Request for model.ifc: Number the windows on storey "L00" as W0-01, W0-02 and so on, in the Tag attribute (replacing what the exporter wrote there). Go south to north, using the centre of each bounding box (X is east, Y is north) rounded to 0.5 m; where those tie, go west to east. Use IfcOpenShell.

First a look at what the model holds.

```python
import ifcopenshell
import ifcopenshell.util.element
import ifcopenshell.util.placement

model = ifcopenshell.open("model.ifc")
print(model.schema)
storey = next(s for s in model.by_type("IfcBuildingStorey") if s.Name == "L00")
windows = [e for e in ifcopenshell.util.element.get_decomposition(storey) if e.is_a("IfcWindow")]
for e in sorted(windows, key=lambda e: e.id()):
    origin = ifcopenshell.util.placement.get_local_placement(e.ObjectPlacement)[:3, 3]
    print(e.id(), e.Tag, e.Name, origin.round(2) + 0.0, sep=" | ")
```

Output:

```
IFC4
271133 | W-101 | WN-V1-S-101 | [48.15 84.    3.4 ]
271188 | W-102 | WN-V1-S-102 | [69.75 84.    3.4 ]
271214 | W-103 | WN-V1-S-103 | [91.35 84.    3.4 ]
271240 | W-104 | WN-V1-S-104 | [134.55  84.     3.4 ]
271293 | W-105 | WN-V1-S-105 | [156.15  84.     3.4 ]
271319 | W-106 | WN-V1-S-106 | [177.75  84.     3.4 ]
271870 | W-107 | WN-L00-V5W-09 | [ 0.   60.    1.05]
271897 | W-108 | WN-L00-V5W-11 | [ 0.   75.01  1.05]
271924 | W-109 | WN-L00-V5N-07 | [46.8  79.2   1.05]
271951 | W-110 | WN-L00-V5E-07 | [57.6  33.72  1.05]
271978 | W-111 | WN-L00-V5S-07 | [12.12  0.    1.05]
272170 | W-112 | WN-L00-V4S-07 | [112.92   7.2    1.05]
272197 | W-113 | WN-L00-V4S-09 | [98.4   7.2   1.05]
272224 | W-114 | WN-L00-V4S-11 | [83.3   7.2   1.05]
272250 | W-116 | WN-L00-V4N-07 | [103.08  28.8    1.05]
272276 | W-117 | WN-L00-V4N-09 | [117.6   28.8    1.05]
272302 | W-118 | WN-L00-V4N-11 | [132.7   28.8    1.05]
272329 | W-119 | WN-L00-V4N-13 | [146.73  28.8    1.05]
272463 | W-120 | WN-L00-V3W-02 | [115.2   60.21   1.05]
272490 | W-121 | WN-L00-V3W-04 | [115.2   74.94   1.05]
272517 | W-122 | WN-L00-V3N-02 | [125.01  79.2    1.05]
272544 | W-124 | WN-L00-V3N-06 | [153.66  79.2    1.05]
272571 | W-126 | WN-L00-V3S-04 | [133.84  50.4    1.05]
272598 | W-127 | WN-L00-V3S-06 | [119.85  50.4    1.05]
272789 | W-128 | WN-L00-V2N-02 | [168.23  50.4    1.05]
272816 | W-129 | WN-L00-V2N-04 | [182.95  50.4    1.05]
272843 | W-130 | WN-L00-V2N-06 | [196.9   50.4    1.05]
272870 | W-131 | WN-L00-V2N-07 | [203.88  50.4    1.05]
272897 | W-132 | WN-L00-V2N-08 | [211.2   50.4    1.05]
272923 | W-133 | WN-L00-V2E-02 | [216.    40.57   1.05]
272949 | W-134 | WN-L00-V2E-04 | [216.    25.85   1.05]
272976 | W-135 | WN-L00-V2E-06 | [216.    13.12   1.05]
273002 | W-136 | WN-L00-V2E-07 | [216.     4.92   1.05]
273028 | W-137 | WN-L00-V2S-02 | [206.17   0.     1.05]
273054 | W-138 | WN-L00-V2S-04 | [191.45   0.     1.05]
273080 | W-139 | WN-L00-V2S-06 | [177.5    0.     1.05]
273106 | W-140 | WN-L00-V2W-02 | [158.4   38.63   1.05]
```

```python
import ifcopenshell
import ifcopenshell.geom
import ifcopenshell.util.element
import ifcopenshell.util.shape

model = ifcopenshell.open("model.ifc")
settings = ifcopenshell.geom.settings()
settings.set("use-world-coords", True)


def centre(element):
    shape = ifcopenshell.geom.create_shape(settings, element)
    return ifcopenshell.util.shape.get_bbox_centroid(shape.geometry)


storey = next(s for s in model.by_type("IfcBuildingStorey") if s.Name == "L00")
windows = [e for e in ifcopenshell.util.element.get_decomposition(storey) if e.is_a("IfcWindow")]

# Insertion points can sit at a corner or the storey origin, so sort by the geometry (in metres).
centres = {e: centre(e) for e in windows}
windows.sort(key=lambda e: (round(centres[e][1] / 0.5), centres[e][0]))

for i, e in enumerate(windows, start=1):
    number = f"W0-{i:02d}"
    e.Tag = number
    print(e.id(), number)

model.write("model-out.ifc")
```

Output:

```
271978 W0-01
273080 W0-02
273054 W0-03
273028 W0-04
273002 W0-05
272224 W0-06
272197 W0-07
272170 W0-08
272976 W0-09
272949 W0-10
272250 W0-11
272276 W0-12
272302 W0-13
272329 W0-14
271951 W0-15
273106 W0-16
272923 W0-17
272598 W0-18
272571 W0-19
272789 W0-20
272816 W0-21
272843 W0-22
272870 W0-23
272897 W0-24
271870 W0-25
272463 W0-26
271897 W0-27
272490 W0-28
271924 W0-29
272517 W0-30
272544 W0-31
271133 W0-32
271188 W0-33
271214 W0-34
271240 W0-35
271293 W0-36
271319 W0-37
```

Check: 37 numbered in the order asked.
